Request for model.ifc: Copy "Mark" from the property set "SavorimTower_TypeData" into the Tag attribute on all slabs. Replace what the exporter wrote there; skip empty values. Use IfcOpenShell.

First a look at what the model holds.

```python
import ifcopenshell
import ifcopenshell.util.element

model = ifcopenshell.open("model.ifc")
print(model.schema)
slabs = model.by_type("IfcSlab")
print(len(slabs), "slabs")
for e in slabs[:8]:
    source = ifcopenshell.util.element.get_pset(e, "SavorimTower_TypeData", "Mark")
    target = e.Tag
    print(e.id(), repr(source), repr(target), sep=" | ")
```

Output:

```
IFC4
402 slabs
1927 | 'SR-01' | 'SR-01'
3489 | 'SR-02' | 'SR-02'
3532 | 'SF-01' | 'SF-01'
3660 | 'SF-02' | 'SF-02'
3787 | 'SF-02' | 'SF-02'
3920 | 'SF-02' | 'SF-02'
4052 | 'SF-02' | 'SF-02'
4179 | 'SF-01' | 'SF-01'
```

```python
import ifcopenshell
import ifcopenshell.util.element

model = ifcopenshell.open("model.ifc")

count = 0
for e in model.by_type("IfcSlab"):
    value = ifcopenshell.util.element.get_pset(e, "SavorimTower_TypeData", "Mark")
    current = e.Tag
    if not value or not value.strip() or current == value:
        continue
    e.Tag = value
    count += 1

print(count, "slabs updated")

model.write("model_edited.ifc")
```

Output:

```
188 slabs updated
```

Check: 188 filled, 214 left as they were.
